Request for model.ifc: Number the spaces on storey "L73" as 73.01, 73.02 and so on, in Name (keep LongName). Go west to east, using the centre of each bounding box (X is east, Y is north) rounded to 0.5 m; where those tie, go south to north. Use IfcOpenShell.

First a look at what the model holds.

```python
import ifcopenshell
import ifcopenshell.util.element
import ifcopenshell.util.placement

model = ifcopenshell.open("model.ifc")
print(model.schema)
storey = next(s for s in model.by_type("IfcBuildingStorey") if s.Name == "L73")
spaces = [e for e in ifcopenshell.util.element.get_decomposition(storey) if e.is_a("IfcSpace")]
for e in sorted(spaces, key=lambda e: e.id()):
    origin = ifcopenshell.util.placement.get_local_placement(e.ObjectPlacement)[:3, 3]
    print(e.id(), e.Name, e.LongName, origin.round(2) + 0.0, sep=" | ")
```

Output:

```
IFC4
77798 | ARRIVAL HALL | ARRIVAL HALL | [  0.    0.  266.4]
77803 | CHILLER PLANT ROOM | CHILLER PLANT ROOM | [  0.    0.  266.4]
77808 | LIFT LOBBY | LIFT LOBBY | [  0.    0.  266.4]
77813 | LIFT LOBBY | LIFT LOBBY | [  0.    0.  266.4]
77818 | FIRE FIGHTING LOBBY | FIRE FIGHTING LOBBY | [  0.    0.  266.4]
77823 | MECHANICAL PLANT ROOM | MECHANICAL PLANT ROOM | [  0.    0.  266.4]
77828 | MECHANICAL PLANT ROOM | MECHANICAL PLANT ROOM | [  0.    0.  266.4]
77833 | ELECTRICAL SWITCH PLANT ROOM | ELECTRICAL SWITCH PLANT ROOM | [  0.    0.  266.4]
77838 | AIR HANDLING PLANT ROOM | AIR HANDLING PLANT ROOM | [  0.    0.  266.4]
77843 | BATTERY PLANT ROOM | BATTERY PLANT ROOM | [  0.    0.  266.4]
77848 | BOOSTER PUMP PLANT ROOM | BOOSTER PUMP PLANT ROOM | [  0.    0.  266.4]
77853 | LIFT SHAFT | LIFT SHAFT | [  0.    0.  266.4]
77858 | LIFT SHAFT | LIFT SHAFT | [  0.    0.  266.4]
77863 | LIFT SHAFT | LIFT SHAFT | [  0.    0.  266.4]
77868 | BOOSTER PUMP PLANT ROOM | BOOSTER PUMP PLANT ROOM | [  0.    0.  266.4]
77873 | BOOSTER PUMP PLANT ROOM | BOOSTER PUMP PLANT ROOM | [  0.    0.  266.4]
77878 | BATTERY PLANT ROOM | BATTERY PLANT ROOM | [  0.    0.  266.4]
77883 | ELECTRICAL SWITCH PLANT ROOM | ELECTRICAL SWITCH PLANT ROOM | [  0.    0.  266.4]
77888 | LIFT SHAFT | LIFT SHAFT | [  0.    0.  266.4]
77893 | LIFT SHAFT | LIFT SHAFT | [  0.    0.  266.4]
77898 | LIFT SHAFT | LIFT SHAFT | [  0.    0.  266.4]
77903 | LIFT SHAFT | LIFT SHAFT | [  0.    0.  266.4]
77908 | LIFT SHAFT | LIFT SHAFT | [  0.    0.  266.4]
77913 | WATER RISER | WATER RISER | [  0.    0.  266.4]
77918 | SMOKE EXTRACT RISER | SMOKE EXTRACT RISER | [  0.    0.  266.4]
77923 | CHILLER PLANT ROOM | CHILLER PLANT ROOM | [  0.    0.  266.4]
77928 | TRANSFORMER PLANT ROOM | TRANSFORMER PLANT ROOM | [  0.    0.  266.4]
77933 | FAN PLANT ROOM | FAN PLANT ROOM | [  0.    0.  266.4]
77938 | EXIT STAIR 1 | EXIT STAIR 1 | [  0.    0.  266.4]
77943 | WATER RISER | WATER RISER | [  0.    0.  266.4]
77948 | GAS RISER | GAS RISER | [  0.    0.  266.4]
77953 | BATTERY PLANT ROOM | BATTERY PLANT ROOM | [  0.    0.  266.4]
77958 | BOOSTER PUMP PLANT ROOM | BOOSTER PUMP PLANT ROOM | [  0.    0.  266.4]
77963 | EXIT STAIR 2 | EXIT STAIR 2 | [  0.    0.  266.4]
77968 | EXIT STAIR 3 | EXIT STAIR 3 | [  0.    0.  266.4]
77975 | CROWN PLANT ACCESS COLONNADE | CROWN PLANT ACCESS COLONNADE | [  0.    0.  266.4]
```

```python
import ifcopenshell
import ifcopenshell.geom
import ifcopenshell.util.element
import ifcopenshell.util.shape

model = ifcopenshell.open("model.ifc")
settings = ifcopenshell.geom.settings()
settings.set("use-world-coords", True)


def centre(element):
    shape = ifcopenshell.geom.create_shape(settings, element)
    return ifcopenshell.util.shape.get_bbox_centroid(shape.geometry)


storey = next(s for s in model.by_type("IfcBuildingStorey") if s.Name == "L73")
spaces = [e for e in ifcopenshell.util.element.get_decomposition(storey) if e.is_a("IfcSpace")]

# Insertion points can sit at a corner or the storey origin, so sort by the geometry (in metres).
centres = {e: centre(e) for e in spaces}
spaces.sort(key=lambda e: (round(centres[e][0] / 0.5), centres[e][1]))

for i, e in enumerate(spaces, start=1):
    number = f"73.{i:02d}"
    e.Name = number
    print(e.id(), number)

model.write("model-out.ifc")
```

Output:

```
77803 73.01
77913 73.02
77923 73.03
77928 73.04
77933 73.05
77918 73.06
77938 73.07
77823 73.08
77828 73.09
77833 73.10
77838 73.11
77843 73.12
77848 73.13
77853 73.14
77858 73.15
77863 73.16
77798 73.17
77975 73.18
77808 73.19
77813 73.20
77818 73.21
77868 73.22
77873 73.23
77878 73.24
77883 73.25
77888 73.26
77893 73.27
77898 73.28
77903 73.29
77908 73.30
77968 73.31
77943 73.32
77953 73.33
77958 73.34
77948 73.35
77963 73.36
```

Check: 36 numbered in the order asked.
